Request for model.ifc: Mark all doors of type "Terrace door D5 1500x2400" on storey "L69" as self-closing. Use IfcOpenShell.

First a look at what the model holds.

```python
import ifcopenshell
import ifcopenshell.util.element

model = ifcopenshell.open("model.ifc")
print(model.schema)
storey = next(s for s in model.by_type("IfcBuildingStorey") if s.Name == "L69")
doors = [e for e in ifcopenshell.util.element.get_decomposition(storey) if e.is_a("IfcDoor")]
seen = {}
for e in doors:
    element_type = ifcopenshell.util.element.get_type(e)
    key = (element_type.Name if element_type != e and element_type else None, ifcopenshell.util.element.get_pset(e, "Pset_DoorCommon", "SelfClosing"))
    seen[key] = seen.get(key, 0) + 1
for (name, value), count in sorted(seen.items(), key=str):
    print(count, "x", name, "|", value)
```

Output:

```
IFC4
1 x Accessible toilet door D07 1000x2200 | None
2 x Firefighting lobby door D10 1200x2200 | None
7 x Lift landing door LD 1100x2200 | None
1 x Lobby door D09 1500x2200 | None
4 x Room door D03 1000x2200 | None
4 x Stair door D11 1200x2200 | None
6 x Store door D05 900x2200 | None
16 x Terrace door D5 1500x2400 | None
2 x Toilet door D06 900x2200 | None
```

```python
import ifcopenshell
import ifcopenshell.api.pset
import ifcopenshell.util.element

model = ifcopenshell.open("model.ifc")

storey = next(s for s in model.by_type("IfcBuildingStorey") if s.Name == "L69")
doors = [e for e in ifcopenshell.util.element.get_decomposition(storey) if e.is_a("IfcDoor")]

count = 0
for e in doors:
    element_type = ifcopenshell.util.element.get_type(e)
    if element_type in (None, e) or element_type.Name != "Terrace door D5 1500x2400":
        continue
    # add_pset returns the element's existing set when there is one.
    pset = ifcopenshell.api.pset.add_pset(model, product=e, name="Pset_DoorCommon")
    ifcopenshell.api.pset.edit_pset(model, pset=pset, properties={"SelfClosing": True})
    count += 1

print(count, "doors updated")

model.write("model_rev.ifc")
```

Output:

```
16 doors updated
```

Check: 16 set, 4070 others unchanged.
